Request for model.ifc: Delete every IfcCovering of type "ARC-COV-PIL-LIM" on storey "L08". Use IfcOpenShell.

First a look at what the model holds.

```python
import ifcopenshell
import ifcopenshell.util.element

model = ifcopenshell.open("model.ifc")
print(model.schema)
storey = next(s for s in model.by_type("IfcBuildingStorey") if s.Name == "L08")
coverings = [e for e in ifcopenshell.util.element.get_decomposition(storey) if e.is_a("IfcCovering")]
seen = {}
for e in coverings:
    element_type = ifcopenshell.util.element.get_type(e)
    name = element_type.Name if element_type not in (None, e) else None
    seen[name] = seen.get(name, 0) + 1
for name, count in sorted(seen.items(), key=str):
    print(count, "x", name)
```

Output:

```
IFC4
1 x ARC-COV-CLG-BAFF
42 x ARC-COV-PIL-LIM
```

```python
import ifcopenshell
import ifcopenshell.api.root
import ifcopenshell.util.element

model = ifcopenshell.open("model.ifc")

storey = next(s for s in model.by_type("IfcBuildingStorey") if s.Name == "L08")
coverings = [e for e in ifcopenshell.util.element.get_decomposition(storey) if e.is_a("IfcCovering")]
targets = [e for e in coverings if (t := ifcopenshell.util.element.get_type(e)) not in (None, e) and t.Name == "ARC-COV-PIL-LIM"]

for e in targets:
    ifcopenshell.api.root.remove_product(model, product=e)
print(len(targets), "removed")

model.write("model_updated.ifc")
```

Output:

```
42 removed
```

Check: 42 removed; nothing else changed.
